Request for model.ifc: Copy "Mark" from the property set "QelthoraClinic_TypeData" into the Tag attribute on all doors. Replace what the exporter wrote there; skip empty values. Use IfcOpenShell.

First a look at what the model holds.

```python
import ifcopenshell
import ifcopenshell.util.element

model = ifcopenshell.open("model.ifc")
print(model.schema)
doors = model.by_type("IfcDoor")
print(len(doors), "doors")
for e in doors[:8]:
    source = ifcopenshell.util.element.get_pset(e, "QelthoraClinic_TypeData", "Mark")
    target = e.Tag
    print(e.id(), repr(source), repr(target), sep=" | ")
```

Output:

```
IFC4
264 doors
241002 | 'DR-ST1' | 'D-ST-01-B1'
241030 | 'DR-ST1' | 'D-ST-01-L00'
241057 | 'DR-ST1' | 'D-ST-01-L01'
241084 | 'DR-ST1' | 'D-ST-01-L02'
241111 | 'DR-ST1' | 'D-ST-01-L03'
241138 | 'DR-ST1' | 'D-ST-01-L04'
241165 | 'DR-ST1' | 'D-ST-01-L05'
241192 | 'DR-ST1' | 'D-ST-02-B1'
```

```python
import ifcopenshell
import ifcopenshell.util.element

model = ifcopenshell.open("model.ifc")

count = 0
for e in model.by_type("IfcDoor"):
    value = ifcopenshell.util.element.get_pset(e, "QelthoraClinic_TypeData", "Mark")
    current = e.Tag
    if not value or not value.strip() or current == value:
        continue
    e.Tag = value
    count += 1

print(count, "doors updated")

model.write("model-out.ifc")
```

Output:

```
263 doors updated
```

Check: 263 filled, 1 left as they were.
